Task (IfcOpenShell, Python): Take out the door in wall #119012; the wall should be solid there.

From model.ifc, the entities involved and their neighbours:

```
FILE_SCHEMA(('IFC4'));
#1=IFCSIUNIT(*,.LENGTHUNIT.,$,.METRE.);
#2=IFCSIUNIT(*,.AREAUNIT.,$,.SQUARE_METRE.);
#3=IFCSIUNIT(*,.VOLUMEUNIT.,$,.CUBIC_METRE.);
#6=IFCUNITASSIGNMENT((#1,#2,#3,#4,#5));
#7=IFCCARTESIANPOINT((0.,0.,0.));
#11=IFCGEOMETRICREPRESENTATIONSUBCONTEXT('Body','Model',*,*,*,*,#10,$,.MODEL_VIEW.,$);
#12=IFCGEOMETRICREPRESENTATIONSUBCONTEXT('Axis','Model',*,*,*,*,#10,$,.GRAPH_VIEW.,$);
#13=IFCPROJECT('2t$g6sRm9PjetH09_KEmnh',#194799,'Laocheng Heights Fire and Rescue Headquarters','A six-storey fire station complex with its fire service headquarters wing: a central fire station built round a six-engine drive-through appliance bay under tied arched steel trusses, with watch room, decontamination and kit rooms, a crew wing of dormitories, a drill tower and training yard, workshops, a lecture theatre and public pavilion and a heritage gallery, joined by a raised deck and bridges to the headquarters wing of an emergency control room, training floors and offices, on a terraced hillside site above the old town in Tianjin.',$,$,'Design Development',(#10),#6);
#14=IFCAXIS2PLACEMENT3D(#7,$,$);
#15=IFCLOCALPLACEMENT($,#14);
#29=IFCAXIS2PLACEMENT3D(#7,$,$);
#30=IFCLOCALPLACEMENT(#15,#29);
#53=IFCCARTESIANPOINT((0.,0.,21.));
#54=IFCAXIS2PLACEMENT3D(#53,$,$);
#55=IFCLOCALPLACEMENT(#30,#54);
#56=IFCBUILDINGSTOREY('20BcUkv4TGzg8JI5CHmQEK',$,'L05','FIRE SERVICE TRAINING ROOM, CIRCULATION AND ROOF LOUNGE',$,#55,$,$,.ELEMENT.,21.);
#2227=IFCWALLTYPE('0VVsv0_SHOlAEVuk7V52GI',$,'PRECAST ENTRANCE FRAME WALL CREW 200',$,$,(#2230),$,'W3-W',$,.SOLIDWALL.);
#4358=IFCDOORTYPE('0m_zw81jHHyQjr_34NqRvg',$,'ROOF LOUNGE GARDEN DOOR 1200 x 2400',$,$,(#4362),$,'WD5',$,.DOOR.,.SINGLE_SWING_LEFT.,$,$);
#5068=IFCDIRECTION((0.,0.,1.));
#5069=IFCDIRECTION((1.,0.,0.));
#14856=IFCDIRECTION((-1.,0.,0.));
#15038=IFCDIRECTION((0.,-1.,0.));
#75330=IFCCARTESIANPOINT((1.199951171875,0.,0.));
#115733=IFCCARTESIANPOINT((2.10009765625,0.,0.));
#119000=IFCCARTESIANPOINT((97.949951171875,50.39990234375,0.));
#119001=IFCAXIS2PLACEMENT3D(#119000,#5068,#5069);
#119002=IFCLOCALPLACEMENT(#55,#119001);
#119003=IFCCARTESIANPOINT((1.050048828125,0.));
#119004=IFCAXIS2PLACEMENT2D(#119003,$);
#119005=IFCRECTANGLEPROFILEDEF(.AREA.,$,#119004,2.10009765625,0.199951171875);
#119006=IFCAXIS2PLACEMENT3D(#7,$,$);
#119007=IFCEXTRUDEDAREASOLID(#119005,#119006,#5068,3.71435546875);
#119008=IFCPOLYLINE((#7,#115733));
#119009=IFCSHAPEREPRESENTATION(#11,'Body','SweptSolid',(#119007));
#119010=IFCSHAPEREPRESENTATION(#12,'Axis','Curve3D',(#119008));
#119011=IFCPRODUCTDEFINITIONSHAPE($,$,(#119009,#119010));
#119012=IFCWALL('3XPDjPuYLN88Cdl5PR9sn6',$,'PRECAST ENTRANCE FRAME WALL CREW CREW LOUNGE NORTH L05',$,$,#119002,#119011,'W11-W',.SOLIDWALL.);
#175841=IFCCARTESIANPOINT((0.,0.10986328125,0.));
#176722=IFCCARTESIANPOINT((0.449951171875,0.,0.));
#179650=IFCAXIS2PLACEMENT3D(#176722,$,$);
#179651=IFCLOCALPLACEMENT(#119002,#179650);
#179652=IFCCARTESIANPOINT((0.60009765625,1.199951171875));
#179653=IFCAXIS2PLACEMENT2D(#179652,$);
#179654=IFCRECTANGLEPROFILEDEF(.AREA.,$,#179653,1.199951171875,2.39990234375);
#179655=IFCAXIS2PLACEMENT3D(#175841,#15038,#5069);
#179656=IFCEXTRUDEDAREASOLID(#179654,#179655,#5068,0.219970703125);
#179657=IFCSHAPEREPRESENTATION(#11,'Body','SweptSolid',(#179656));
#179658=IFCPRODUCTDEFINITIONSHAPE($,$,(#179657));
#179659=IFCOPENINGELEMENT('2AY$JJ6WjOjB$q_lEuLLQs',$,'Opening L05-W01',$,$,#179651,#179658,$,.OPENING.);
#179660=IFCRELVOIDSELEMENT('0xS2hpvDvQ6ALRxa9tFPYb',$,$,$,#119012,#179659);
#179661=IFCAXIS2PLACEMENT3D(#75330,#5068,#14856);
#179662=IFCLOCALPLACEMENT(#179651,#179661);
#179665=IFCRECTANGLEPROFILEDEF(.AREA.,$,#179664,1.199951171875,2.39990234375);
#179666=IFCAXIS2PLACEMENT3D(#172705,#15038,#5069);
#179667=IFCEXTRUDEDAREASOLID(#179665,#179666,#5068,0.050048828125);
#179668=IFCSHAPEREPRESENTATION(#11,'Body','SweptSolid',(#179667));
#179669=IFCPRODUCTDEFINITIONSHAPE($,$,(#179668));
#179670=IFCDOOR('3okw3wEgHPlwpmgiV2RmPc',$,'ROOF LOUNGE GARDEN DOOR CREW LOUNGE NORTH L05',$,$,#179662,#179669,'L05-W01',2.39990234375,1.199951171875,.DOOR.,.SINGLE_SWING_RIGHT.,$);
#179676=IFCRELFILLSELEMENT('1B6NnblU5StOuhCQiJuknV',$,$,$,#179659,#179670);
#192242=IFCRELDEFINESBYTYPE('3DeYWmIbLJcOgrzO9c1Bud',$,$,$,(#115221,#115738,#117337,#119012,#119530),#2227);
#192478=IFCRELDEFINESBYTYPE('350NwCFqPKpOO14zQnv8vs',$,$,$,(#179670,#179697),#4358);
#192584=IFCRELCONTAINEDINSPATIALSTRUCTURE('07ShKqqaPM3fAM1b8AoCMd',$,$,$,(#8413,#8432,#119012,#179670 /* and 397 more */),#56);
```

```python
import ifcopenshell
import ifcopenshell.api.feature
import ifcopenshell.api.root
import ifcopenshell.geom
import ifcopenshell.util.shape

model = ifcopenshell.open("model.ifc")
settings = ifcopenshell.geom.settings()


def volume(element):
    """Net volume in cubic metres, openings subtracted."""
    shape = ifcopenshell.geom.create_shape(settings, element)
    return ifcopenshell.util.shape.get_volume(shape.geometry)


door = model.by_id(179670)
opening = door.FillsVoids[0].RelatingOpeningElement
wall = opening.VoidsElements[0].RelatingBuildingElement
before = volume(wall)

ifcopenshell.api.root.remove_product(model, product=door)
ifcopenshell.api.feature.remove_feature(model, feature=opening)

after = volume(wall)

print(f"wall volume {before:.3f} -> {after:.3f} m3")

model.write("model_rev.ifc")
```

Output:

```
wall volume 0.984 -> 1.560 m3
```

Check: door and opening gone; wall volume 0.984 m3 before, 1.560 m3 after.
